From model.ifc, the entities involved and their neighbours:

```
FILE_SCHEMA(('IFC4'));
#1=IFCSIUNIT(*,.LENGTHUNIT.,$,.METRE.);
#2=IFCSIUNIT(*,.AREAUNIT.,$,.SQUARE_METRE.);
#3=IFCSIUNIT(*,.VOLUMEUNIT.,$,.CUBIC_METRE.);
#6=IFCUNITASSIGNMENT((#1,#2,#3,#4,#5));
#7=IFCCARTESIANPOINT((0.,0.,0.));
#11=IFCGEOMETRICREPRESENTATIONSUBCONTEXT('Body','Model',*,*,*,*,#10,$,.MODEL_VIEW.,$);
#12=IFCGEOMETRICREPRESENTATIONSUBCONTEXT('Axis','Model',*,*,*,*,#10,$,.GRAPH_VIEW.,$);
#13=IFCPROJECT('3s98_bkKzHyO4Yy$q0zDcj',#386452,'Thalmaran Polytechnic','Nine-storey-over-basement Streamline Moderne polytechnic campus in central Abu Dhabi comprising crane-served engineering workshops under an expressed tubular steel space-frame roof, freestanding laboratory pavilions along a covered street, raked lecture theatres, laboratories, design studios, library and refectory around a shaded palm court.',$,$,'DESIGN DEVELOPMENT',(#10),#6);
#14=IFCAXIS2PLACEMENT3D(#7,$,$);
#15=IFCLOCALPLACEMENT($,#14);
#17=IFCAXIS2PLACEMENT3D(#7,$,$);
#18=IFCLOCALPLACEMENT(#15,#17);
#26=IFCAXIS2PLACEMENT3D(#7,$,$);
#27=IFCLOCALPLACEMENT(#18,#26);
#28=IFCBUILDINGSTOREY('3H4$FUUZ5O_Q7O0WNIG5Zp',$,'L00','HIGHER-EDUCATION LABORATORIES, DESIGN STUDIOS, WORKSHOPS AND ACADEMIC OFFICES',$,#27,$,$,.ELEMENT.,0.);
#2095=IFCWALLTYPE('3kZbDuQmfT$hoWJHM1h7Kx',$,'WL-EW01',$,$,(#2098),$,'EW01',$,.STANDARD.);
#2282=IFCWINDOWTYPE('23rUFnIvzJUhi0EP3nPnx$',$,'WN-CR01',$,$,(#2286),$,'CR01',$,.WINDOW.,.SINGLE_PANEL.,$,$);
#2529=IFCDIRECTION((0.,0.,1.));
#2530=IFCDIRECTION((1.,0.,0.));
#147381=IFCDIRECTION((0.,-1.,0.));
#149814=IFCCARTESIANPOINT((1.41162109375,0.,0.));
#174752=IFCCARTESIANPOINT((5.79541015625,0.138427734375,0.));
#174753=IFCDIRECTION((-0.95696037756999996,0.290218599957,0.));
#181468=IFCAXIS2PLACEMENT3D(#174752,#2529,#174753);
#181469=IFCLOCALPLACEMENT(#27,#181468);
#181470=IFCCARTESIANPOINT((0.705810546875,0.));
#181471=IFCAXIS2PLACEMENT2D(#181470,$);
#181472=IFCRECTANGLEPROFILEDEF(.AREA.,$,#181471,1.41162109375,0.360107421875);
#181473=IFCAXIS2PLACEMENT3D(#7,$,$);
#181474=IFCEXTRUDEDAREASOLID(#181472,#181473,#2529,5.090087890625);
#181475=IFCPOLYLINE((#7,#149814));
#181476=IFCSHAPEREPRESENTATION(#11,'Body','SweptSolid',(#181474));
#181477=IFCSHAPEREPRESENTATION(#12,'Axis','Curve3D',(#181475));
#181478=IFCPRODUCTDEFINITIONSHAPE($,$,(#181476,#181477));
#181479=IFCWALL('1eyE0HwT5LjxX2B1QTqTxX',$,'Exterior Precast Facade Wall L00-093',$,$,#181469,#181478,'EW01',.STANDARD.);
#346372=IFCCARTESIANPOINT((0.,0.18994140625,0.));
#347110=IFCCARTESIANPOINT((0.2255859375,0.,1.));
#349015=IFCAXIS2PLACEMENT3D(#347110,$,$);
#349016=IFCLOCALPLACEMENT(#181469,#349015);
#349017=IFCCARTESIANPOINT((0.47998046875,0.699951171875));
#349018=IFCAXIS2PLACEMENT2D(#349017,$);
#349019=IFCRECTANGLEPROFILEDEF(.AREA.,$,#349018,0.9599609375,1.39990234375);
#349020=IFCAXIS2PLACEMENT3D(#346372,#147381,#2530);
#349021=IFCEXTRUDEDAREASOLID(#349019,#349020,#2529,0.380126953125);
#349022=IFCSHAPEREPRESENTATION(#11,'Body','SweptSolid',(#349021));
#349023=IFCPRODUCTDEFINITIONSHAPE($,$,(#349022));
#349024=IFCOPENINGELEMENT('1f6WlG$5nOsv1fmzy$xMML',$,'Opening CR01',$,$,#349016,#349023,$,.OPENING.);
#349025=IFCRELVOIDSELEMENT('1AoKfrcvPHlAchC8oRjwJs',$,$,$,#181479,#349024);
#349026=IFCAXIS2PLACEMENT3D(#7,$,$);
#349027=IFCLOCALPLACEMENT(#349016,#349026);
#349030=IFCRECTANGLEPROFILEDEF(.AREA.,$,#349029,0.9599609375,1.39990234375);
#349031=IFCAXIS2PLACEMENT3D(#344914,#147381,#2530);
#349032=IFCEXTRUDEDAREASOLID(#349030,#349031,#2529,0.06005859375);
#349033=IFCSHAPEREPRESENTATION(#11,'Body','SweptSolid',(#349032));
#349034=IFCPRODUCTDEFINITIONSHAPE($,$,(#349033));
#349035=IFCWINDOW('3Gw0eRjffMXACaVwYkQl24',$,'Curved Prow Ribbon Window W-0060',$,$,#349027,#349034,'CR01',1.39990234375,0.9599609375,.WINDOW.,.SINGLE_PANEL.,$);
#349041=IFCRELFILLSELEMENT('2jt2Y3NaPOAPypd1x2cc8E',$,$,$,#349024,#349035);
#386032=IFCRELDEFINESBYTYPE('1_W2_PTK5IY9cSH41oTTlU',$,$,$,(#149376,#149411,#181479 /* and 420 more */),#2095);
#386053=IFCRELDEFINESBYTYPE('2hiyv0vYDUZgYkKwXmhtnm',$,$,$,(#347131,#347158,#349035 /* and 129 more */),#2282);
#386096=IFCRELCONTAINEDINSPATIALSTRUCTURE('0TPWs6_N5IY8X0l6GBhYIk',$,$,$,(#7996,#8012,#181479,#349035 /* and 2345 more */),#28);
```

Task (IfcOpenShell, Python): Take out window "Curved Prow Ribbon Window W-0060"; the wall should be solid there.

```python
import ifcopenshell
import ifcopenshell.api.feature
import ifcopenshell.api.root
import ifcopenshell.geom
import ifcopenshell.util.shape

model = ifcopenshell.open("model.ifc")
settings = ifcopenshell.geom.settings()


def volume(element):
    """Net volume in cubic metres, openings subtracted."""
    shape = ifcopenshell.geom.create_shape(settings, element)
    return ifcopenshell.util.shape.get_volume(shape.geometry)


window = model.by_guid("3Gw0eRjffMXACaVwYkQl24")
opening = window.FillsVoids[0].RelatingOpeningElement
wall = opening.VoidsElements[0].RelatingBuildingElement
before = volume(wall)

ifcopenshell.api.root.remove_product(model, product=window)
ifcopenshell.api.feature.remove_feature(model, feature=opening)

after = volume(wall)

print(f"wall volume {before:.3f} -> {after:.3f} m3")

model.write("model_rev.ifc")
```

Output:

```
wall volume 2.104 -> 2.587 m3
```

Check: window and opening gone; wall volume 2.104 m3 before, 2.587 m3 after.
